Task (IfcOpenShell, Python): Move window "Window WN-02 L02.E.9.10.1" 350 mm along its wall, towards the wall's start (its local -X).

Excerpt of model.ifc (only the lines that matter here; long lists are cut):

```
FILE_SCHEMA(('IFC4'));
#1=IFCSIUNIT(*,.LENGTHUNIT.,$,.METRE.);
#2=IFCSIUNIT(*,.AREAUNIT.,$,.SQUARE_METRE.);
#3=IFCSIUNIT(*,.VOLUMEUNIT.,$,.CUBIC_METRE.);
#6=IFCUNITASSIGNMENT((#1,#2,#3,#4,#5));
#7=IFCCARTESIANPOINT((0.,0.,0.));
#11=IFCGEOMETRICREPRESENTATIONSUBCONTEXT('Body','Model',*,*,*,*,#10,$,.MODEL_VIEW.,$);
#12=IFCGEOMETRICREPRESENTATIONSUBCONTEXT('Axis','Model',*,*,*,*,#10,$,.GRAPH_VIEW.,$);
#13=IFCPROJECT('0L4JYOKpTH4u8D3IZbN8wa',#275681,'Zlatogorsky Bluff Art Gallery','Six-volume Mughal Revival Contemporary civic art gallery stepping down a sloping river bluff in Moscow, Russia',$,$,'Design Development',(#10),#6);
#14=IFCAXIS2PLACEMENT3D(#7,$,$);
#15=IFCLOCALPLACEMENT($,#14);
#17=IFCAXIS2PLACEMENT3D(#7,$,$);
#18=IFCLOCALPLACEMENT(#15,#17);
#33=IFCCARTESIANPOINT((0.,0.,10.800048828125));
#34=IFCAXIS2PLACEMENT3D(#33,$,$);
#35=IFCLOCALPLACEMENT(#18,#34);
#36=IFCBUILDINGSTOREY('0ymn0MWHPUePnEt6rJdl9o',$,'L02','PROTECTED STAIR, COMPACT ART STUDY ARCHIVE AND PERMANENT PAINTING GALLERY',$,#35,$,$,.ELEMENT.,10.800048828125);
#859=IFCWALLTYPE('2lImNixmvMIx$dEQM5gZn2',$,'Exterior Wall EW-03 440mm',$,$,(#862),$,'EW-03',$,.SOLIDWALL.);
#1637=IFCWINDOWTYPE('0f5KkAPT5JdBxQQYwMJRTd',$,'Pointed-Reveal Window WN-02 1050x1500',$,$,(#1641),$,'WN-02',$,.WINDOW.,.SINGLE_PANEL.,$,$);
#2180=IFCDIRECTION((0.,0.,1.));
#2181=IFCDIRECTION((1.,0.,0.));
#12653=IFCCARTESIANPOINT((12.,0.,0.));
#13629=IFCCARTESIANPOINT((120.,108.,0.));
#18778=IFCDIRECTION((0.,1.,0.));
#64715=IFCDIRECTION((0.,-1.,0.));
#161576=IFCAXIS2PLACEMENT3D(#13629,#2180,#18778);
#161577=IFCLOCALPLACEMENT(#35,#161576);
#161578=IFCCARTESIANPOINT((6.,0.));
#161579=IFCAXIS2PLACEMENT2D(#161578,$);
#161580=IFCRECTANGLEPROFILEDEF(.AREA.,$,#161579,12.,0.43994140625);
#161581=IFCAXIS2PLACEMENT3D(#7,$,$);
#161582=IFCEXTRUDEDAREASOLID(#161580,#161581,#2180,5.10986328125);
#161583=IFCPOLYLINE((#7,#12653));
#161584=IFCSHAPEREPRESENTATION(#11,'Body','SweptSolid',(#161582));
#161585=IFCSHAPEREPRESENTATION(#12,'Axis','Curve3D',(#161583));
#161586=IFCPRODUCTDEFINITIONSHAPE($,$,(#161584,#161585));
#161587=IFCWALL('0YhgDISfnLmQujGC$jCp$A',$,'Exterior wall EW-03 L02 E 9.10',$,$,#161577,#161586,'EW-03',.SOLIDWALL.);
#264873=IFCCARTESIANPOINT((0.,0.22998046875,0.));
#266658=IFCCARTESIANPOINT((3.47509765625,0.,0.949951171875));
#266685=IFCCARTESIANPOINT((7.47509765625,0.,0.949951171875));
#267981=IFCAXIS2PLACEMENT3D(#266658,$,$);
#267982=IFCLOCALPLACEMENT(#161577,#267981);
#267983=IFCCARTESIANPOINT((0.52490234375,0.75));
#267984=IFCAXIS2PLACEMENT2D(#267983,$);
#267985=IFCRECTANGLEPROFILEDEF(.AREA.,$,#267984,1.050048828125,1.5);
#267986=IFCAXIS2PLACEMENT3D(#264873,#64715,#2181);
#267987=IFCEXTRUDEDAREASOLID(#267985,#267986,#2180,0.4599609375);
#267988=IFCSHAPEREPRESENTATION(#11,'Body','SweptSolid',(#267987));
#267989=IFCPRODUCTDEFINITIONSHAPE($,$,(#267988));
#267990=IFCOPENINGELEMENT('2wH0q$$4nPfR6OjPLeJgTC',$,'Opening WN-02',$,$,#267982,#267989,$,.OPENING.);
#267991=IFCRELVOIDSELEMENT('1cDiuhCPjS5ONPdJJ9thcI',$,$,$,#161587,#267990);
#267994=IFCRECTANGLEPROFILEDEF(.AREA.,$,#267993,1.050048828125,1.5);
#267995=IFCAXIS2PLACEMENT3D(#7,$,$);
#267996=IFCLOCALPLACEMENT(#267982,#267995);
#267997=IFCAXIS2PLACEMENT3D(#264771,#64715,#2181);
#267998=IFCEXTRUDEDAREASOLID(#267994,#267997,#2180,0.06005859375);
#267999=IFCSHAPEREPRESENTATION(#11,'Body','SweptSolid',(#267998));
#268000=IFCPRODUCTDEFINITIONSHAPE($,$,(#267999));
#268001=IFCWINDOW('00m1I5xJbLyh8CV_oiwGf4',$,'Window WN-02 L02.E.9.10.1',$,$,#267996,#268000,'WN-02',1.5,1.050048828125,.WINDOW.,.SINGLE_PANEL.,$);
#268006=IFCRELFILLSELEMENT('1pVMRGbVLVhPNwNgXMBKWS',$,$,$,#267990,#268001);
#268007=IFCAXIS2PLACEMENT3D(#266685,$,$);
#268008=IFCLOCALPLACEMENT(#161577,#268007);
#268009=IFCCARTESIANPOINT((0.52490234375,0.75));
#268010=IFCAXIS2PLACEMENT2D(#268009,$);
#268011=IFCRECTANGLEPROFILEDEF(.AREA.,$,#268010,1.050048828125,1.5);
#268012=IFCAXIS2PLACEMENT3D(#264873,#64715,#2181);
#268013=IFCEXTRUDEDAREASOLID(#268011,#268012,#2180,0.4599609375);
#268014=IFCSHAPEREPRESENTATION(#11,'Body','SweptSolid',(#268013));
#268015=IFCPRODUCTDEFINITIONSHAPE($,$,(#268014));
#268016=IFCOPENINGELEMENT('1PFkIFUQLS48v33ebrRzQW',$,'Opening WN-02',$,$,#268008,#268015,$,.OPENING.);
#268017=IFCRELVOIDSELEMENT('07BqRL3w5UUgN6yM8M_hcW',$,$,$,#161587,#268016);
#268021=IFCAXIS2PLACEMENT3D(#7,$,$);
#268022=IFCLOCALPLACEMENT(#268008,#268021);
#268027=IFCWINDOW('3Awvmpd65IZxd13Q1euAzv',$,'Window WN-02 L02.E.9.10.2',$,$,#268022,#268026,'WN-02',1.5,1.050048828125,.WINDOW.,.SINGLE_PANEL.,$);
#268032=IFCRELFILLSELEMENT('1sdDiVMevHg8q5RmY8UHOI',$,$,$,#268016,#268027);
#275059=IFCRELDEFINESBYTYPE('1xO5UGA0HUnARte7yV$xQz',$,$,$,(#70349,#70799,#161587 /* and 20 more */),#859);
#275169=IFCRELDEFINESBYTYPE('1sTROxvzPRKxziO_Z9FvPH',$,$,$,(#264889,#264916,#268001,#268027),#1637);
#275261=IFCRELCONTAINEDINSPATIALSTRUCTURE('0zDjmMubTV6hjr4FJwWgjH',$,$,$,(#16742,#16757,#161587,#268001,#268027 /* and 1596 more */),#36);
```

```python
import ifcopenshell
import ifcopenshell.api.geometry
import ifcopenshell.util.placement
import ifcopenshell.util.unit

model = ifcopenshell.open("model.ifc")
unit_scale = ifcopenshell.util.unit.calculate_unit_scale(model)

window = model.by_id(268001)
opening = window.FillsVoids[0].RelatingOpeningElement
wall = opening.VoidsElements[0].RelatingBuildingElement

wall_matrix = ifcopenshell.util.placement.get_local_placement(wall.ObjectPlacement)
shift = wall_matrix[:3, 0] * -0.35 / unit_scale
before = ifcopenshell.util.placement.get_local_placement(window.ObjectPlacement)[:3, 3].copy()

# The window is placed relative to its opening, so it follows when the opening moves.
matrix = ifcopenshell.util.placement.get_local_placement(opening.ObjectPlacement)
matrix[:3, 3] += shift
ifcopenshell.api.geometry.edit_object_placement(
    model, product=opening, matrix=matrix, is_si=False, should_transform_children=True
)

after = ifcopenshell.util.placement.get_local_placement(window.ObjectPlacement)[:3, 3]
print("window moved by", (after - before).round(3) + 0.0)

model.write("model_edited.ifc")
```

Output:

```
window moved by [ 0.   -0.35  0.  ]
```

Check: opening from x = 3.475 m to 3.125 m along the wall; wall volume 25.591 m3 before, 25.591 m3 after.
